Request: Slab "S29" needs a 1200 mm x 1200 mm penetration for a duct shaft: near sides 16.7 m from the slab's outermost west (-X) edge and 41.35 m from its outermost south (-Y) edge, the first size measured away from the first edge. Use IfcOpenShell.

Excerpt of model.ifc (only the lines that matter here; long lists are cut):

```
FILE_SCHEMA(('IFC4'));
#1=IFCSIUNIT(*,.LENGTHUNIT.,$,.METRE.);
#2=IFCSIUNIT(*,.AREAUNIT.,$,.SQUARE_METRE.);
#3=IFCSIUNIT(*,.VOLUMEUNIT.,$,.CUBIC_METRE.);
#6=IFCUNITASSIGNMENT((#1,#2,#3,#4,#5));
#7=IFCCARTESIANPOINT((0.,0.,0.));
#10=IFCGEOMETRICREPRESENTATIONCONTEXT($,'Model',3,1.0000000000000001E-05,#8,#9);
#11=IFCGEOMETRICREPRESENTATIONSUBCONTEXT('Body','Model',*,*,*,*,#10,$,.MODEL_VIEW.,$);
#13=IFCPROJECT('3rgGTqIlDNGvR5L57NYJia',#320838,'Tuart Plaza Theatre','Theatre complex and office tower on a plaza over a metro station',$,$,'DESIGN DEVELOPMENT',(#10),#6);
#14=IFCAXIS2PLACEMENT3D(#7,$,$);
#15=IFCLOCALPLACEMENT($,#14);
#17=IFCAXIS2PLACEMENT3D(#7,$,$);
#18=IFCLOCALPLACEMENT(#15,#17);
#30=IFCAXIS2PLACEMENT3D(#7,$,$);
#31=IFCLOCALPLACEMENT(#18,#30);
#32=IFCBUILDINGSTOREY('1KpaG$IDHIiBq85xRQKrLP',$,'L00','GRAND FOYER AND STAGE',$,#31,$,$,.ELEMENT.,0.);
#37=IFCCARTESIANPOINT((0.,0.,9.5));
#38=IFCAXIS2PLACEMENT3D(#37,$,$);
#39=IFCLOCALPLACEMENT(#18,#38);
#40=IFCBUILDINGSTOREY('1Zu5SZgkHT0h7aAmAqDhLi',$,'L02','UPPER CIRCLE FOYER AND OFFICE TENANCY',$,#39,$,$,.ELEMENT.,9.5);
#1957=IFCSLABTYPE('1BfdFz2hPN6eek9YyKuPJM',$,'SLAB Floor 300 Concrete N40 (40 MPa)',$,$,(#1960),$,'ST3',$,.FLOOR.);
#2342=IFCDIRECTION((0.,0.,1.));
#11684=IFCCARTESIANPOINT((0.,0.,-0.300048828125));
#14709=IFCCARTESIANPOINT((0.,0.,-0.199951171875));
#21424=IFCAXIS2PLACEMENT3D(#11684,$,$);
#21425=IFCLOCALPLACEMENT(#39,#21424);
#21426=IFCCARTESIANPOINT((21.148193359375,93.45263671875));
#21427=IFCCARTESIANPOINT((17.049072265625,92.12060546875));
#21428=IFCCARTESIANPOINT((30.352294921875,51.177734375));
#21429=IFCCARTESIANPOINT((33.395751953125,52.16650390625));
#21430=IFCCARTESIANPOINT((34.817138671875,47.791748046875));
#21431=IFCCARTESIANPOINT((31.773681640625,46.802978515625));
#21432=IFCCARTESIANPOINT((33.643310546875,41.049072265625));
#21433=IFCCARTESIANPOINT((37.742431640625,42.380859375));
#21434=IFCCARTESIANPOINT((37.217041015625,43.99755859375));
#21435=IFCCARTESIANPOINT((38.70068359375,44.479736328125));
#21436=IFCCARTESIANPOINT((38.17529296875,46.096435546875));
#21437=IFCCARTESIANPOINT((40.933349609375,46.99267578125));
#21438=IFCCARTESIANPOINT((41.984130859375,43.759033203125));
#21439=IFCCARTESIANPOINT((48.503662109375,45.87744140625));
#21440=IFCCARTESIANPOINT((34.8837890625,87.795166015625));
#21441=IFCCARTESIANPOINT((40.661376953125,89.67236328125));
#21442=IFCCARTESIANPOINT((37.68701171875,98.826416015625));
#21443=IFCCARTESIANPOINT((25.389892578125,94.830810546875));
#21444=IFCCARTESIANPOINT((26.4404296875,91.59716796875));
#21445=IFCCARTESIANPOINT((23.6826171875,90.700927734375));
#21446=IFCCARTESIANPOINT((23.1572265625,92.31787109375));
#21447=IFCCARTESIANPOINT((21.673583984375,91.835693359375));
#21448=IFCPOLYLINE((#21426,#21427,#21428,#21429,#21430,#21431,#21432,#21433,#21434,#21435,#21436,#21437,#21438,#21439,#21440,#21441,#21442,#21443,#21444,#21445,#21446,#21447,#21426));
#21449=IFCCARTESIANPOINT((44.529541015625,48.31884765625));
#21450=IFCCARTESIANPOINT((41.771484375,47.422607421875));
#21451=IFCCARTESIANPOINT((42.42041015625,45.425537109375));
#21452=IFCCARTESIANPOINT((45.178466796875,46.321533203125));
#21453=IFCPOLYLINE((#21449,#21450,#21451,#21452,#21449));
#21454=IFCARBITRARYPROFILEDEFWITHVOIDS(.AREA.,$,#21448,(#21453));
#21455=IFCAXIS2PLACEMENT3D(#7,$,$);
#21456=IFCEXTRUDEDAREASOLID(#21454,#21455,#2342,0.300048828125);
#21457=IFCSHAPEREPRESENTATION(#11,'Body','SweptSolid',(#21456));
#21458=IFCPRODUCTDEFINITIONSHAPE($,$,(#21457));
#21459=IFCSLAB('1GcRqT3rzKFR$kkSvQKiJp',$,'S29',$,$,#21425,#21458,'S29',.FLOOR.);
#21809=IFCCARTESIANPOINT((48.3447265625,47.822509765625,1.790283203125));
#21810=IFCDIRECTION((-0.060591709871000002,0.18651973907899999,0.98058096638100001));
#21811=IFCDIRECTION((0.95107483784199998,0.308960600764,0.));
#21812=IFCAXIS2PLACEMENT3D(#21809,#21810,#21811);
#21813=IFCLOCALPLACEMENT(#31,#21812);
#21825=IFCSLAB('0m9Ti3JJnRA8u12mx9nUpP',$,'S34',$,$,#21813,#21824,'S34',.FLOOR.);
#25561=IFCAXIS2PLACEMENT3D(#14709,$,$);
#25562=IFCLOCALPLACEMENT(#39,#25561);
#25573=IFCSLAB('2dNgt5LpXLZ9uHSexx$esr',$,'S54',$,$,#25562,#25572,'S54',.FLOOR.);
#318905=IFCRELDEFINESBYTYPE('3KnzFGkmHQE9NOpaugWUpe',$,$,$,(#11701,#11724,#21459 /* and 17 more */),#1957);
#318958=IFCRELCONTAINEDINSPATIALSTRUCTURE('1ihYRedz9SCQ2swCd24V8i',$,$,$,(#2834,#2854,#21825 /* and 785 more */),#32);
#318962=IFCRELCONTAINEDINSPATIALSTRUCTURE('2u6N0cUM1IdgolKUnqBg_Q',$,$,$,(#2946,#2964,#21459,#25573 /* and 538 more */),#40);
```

```python
import numpy as np
import ifcopenshell
import ifcopenshell.api.feature
import ifcopenshell.api.geometry
import ifcopenshell.api.root
import ifcopenshell.geom
import ifcopenshell.util.placement
import ifcopenshell.util.representation
import ifcopenshell.util.shape
import ifcopenshell.util.unit

model = ifcopenshell.open("model.ifc")
unit_scale = ifcopenshell.util.unit.calculate_unit_scale(model)
settings = ifcopenshell.geom.settings()


def volume(element):
    """Net volume in cubic metres, openings subtracted."""
    shape = ifcopenshell.geom.create_shape(settings, element)
    return ifcopenshell.util.shape.get_volume(shape.geometry)


slab = model.by_guid("1GcRqT3rzKFR$kkSvQKiJp")
before = volume(slab)

# Extent in the slab's own axes, in metres. The edges named are its -X and -Y sides.
slab_shape = ifcopenshell.geom.create_shape(settings, slab)
vertices = ifcopenshell.util.shape.get_vertices(slab_shape.geometry)
x_min, y_min, bottom = vertices.min(axis=0)
top = vertices[:, 2].max()

opening = ifcopenshell.api.root.create_entity(model, ifc_class="IfcOpeningElement", name="Duct shaft opening", predefined_type="OPENING")
context = ifcopenshell.util.representation.get_context(model, "Model", "Body", "MODEL_VIEW")
width, depth = 1.2, 1.2
outline = [(0.0, 0.0), (width, 0.0), (width, depth), (0.0, depth), (0.0, 0.0)]
# Overshoot both faces by 50 mm so the cut is clean.
shape = ifcopenshell.api.geometry.add_slab_representation(
    model, context=context, depth=top - bottom + 0.1, polyline=outline
)
ifcopenshell.api.geometry.assign_representation(model, product=opening, representation=shape)

matrix = ifcopenshell.util.placement.get_local_placement(slab.ObjectPlacement)
matrix[:, 3] = matrix @ np.append(np.array([x_min + 16.7, y_min + 41.35, bottom - 0.05]) / unit_scale, 1.0)
ifcopenshell.api.geometry.edit_object_placement(model, product=opening, matrix=matrix, is_si=False)
ifcopenshell.api.feature.add_feature(model, feature=opening, element=slab)

after = volume(slab)

print(f"slab volume {before:.3f} -> {after:.3f} m3")

model.write("model_updated.ifc")
```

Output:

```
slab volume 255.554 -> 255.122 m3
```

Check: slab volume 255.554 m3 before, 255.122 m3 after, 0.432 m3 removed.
